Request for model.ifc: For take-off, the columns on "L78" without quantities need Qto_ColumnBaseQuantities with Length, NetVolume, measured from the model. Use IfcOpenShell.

First a look at what the model holds.

```python
import ifcopenshell
import ifcopenshell.util.element
import ifcopenshell.util.unit

model = ifcopenshell.open("model.ifc")
print(model.schema)
for unit_type in ("LENGTHUNIT", "AREAUNIT", "VOLUMEUNIT"):
    print(unit_type, ifcopenshell.util.unit.calculate_unit_scale(model, unit_type))
storey = next(s for s in model.by_type("IfcBuildingStorey") if s.Name == "L78")
columns = [e for e in ifcopenshell.util.element.get_decomposition(storey) if e.is_a("IfcColumn")]
for e in sorted(columns, key=lambda e: e.id()):
    print(e.id(), e.is_a(), e.Name, list(ifcopenshell.util.element.get_psets(e, qtos_only=True)), sep=" | ")
```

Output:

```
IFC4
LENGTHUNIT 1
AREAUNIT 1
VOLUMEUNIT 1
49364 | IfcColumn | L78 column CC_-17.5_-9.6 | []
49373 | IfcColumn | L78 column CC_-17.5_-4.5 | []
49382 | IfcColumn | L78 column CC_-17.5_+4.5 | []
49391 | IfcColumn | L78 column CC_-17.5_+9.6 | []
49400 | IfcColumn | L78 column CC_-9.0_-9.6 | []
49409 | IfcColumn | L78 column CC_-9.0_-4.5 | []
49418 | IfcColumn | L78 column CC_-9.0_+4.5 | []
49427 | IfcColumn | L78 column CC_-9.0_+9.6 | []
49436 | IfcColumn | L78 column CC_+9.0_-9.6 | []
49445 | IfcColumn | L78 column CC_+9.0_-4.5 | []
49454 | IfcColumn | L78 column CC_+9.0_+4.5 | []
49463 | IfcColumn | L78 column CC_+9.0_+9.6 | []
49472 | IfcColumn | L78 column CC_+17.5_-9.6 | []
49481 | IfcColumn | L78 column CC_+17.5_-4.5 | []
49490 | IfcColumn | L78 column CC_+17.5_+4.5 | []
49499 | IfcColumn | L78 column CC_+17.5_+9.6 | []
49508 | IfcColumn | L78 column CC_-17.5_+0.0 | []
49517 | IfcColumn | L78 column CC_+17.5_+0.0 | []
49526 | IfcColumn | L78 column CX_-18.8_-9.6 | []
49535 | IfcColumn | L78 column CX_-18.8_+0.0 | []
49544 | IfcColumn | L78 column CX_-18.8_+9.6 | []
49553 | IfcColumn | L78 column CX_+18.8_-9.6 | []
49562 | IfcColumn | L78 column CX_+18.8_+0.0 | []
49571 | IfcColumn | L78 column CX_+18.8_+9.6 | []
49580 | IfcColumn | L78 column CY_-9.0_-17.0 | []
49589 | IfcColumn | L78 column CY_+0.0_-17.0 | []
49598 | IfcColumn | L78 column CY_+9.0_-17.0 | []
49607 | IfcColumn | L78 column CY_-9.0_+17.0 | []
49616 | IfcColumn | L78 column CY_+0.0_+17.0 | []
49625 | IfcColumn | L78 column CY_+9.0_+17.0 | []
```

```python
import ifcopenshell
import ifcopenshell.api.pset
import ifcopenshell.geom
import ifcopenshell.util.element
import ifcopenshell.util.shape
import ifcopenshell.util.unit

model = ifcopenshell.open("model.ifc")
unit_scale = ifcopenshell.util.unit.calculate_unit_scale(model)
volume_scale = ifcopenshell.util.unit.calculate_unit_scale(model, "VOLUMEUNIT")
settings = ifcopenshell.geom.settings()

storey = next(s for s in model.by_type("IfcBuildingStorey") if s.Name == "L78")
columns = [e for e in ifcopenshell.util.element.get_decomposition(storey) if e.is_a("IfcColumn")]

for e in sorted(columns, key=lambda e: e.id()):
    if ifcopenshell.util.element.get_psets(e, qtos_only=True, should_inherit=False):
        continue
    # Geometry comes back in metres, in the element's own axes.
    shape = ifcopenshell.geom.create_shape(settings, e)
    values = {
        "Length": ifcopenshell.util.shape.get_z(shape.geometry) / unit_scale,
        "NetVolume": ifcopenshell.util.shape.get_volume(shape.geometry) / volume_scale,
    }
    qto = ifcopenshell.api.pset.add_qto(model, product=e, name="Qto_ColumnBaseQuantities")
    ifcopenshell.api.pset.edit_qto(model, qto=qto, properties=values)
    print(e.id(), {k: round(v, 3) for k, v in values.items()})

model.write("model_v2.ifc")
```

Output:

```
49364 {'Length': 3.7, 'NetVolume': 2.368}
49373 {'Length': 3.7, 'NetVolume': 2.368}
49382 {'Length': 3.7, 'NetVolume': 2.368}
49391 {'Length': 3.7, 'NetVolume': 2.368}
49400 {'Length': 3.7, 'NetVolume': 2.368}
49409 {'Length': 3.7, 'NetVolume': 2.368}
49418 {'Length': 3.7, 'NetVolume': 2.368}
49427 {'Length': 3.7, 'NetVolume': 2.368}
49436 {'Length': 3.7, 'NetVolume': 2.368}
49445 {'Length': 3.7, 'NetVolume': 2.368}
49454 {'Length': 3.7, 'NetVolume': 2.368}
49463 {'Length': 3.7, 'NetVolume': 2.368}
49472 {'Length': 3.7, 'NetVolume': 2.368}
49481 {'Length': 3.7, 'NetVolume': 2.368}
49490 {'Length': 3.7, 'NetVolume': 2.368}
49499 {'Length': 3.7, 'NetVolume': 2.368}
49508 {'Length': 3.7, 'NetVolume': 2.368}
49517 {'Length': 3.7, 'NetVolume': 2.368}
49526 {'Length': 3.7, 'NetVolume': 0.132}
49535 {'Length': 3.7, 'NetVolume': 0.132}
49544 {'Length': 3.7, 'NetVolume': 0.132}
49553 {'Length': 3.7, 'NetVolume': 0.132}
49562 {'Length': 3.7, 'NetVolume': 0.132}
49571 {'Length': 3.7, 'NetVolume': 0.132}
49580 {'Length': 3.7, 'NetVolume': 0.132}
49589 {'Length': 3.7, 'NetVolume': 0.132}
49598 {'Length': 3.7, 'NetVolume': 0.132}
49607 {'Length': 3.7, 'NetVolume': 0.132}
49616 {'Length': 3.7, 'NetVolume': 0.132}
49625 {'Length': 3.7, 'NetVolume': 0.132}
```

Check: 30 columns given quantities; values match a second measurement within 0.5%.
